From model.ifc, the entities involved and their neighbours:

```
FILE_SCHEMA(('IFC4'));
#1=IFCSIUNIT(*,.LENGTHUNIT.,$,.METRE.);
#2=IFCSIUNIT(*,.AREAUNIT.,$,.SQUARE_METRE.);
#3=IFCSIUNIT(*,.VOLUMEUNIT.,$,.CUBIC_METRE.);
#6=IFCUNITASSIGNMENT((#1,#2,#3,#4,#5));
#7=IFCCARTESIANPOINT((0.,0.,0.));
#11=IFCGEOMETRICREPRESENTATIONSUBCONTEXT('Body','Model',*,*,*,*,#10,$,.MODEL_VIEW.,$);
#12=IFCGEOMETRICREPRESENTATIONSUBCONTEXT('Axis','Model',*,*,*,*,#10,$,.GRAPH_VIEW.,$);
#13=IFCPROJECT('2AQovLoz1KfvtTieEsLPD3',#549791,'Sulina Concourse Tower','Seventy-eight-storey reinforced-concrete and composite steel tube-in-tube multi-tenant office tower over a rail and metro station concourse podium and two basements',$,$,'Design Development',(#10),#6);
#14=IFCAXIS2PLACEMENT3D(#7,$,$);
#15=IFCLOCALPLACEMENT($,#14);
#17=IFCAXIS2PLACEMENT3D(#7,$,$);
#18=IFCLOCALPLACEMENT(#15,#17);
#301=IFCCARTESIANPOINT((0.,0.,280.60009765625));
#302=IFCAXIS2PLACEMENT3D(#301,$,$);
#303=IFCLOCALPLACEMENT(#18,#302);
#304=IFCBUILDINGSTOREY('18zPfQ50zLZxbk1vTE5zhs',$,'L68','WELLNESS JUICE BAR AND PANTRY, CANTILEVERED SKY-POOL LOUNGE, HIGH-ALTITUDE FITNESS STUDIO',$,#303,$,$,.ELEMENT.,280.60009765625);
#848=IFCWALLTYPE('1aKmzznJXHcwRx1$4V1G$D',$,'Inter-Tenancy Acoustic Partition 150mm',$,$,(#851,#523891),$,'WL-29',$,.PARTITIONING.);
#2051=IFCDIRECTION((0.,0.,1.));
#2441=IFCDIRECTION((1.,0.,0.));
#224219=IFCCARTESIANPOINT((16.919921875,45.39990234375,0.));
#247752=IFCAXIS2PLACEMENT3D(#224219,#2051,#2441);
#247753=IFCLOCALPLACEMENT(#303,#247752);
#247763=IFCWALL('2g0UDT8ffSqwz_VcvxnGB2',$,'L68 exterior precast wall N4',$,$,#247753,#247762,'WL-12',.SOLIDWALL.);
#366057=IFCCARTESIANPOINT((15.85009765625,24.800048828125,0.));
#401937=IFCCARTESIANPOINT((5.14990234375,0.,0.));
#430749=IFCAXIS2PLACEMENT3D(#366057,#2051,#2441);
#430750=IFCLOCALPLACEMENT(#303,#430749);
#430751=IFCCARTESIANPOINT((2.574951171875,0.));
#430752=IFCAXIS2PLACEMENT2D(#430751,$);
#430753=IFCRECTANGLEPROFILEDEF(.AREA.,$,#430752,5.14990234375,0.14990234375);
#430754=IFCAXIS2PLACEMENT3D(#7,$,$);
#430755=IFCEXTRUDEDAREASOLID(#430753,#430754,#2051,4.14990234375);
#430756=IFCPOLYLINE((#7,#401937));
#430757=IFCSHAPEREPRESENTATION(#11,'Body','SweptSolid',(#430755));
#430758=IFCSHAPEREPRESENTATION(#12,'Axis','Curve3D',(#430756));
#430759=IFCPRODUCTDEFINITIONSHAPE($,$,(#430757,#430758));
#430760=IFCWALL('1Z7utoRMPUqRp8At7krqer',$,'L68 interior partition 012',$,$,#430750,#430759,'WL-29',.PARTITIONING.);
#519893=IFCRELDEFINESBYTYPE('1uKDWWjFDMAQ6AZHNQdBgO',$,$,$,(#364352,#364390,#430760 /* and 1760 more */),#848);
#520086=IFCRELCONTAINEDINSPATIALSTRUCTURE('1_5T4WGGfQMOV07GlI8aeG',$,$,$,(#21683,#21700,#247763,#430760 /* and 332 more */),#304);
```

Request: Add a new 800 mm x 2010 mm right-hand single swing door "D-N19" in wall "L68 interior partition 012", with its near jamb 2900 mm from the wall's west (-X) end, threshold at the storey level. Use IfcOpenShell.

```python
import numpy as np
import ifcopenshell
import ifcopenshell.api.feature
import ifcopenshell.api.geometry
import ifcopenshell.api.root
import ifcopenshell.api.spatial
import ifcopenshell.geom
import ifcopenshell.util.element
import ifcopenshell.util.placement
import ifcopenshell.util.representation
import ifcopenshell.util.shape
import ifcopenshell.util.unit

model = ifcopenshell.open("model.ifc")
unit_scale = ifcopenshell.util.unit.calculate_unit_scale(model)
settings = ifcopenshell.geom.settings()


def volume(element):
    """Net volume in cubic metres, openings subtracted."""
    shape = ifcopenshell.geom.create_shape(settings, element)
    return ifcopenshell.util.shape.get_volume(shape.geometry)


wall = model.by_guid("1Z7utoRMPUqRp8At7krqer")
storey = ifcopenshell.util.element.get_container(wall, ifc_class="IfcBuildingStorey")
context = ifcopenshell.util.representation.get_context(model, "Model", "Body", "MODEL_VIEW")
before = volume(wall)

width, height, from_end, sill = 0.8, 2.01, 2.9, 0.0  # metres

# The wall runs along its own X axis, and the end named is its -X end.
wall_shape = ifcopenshell.geom.create_shape(settings, wall)
x, y, z = ifcopenshell.util.shape.get_vertices(wall_shape.geometry).T
start = x.min() + from_end
face, thickness = float(y.min()), float(y.max() - y.min())
wall_matrix = ifcopenshell.util.placement.get_local_placement(wall.ObjectPlacement)
level = ifcopenshell.util.placement.get_local_placement(storey.ObjectPlacement)[2, 3]


def in_wall(x, y):
    """Placement at x, y metres in the wall's axes, at sill height."""
    matrix = wall_matrix.copy()
    matrix[:, 3] = wall_matrix @ np.array([x / unit_scale, y / unit_scale, 0.0, 1.0])
    matrix[2, 3] = level + sill / unit_scale
    return matrix


# Opening: a box that overshoots both wall faces by 50 mm.
opening = ifcopenshell.api.root.create_entity(model, ifc_class="IfcOpeningElement", predefined_type="OPENING")
box = ifcopenshell.api.geometry.add_wall_representation(
    model, context=context, length=width, height=height, thickness=thickness + 0.1
)
ifcopenshell.api.geometry.assign_representation(model, product=opening, representation=box)
ifcopenshell.api.geometry.edit_object_placement(model, product=opening, matrix=in_wall(start, face - 0.05), is_si=False)
ifcopenshell.api.feature.add_feature(model, feature=opening, element=wall)

door = ifcopenshell.api.root.create_entity(model, ifc_class="IfcDoor", name="D-N19", predefined_type="DOOR")
door.OverallWidth, door.OverallHeight = width / unit_scale, height / unit_scale
door.OperationType = "SINGLE_SWING_RIGHT"
body = ifcopenshell.api.geometry.add_door_representation(
    model,
    context=context,
    overall_width=door.OverallWidth,
    overall_height=door.OverallHeight,
    operation_type="SINGLE_SWING_RIGHT",
    lining_properties={"LiningDepth": thickness / unit_scale, "ThresholdDepth": thickness / unit_scale},
)
ifcopenshell.api.geometry.assign_representation(model, product=door, representation=body)
ifcopenshell.api.spatial.assign_container(model, products=[door], relating_structure=storey)
ifcopenshell.api.feature.add_filling(model, opening=opening, element=door)

# The lining spans the wall, so the door starts at the wall face.
ifcopenshell.api.geometry.edit_object_placement(model, product=door, matrix=in_wall(start, face), is_si=False)

after = volume(wall)

print(f"wall volume {before:.3f} -> {after:.3f} m3")

model.write("model_updated.ifc")
```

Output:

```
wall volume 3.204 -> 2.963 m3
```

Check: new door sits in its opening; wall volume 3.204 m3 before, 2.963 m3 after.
